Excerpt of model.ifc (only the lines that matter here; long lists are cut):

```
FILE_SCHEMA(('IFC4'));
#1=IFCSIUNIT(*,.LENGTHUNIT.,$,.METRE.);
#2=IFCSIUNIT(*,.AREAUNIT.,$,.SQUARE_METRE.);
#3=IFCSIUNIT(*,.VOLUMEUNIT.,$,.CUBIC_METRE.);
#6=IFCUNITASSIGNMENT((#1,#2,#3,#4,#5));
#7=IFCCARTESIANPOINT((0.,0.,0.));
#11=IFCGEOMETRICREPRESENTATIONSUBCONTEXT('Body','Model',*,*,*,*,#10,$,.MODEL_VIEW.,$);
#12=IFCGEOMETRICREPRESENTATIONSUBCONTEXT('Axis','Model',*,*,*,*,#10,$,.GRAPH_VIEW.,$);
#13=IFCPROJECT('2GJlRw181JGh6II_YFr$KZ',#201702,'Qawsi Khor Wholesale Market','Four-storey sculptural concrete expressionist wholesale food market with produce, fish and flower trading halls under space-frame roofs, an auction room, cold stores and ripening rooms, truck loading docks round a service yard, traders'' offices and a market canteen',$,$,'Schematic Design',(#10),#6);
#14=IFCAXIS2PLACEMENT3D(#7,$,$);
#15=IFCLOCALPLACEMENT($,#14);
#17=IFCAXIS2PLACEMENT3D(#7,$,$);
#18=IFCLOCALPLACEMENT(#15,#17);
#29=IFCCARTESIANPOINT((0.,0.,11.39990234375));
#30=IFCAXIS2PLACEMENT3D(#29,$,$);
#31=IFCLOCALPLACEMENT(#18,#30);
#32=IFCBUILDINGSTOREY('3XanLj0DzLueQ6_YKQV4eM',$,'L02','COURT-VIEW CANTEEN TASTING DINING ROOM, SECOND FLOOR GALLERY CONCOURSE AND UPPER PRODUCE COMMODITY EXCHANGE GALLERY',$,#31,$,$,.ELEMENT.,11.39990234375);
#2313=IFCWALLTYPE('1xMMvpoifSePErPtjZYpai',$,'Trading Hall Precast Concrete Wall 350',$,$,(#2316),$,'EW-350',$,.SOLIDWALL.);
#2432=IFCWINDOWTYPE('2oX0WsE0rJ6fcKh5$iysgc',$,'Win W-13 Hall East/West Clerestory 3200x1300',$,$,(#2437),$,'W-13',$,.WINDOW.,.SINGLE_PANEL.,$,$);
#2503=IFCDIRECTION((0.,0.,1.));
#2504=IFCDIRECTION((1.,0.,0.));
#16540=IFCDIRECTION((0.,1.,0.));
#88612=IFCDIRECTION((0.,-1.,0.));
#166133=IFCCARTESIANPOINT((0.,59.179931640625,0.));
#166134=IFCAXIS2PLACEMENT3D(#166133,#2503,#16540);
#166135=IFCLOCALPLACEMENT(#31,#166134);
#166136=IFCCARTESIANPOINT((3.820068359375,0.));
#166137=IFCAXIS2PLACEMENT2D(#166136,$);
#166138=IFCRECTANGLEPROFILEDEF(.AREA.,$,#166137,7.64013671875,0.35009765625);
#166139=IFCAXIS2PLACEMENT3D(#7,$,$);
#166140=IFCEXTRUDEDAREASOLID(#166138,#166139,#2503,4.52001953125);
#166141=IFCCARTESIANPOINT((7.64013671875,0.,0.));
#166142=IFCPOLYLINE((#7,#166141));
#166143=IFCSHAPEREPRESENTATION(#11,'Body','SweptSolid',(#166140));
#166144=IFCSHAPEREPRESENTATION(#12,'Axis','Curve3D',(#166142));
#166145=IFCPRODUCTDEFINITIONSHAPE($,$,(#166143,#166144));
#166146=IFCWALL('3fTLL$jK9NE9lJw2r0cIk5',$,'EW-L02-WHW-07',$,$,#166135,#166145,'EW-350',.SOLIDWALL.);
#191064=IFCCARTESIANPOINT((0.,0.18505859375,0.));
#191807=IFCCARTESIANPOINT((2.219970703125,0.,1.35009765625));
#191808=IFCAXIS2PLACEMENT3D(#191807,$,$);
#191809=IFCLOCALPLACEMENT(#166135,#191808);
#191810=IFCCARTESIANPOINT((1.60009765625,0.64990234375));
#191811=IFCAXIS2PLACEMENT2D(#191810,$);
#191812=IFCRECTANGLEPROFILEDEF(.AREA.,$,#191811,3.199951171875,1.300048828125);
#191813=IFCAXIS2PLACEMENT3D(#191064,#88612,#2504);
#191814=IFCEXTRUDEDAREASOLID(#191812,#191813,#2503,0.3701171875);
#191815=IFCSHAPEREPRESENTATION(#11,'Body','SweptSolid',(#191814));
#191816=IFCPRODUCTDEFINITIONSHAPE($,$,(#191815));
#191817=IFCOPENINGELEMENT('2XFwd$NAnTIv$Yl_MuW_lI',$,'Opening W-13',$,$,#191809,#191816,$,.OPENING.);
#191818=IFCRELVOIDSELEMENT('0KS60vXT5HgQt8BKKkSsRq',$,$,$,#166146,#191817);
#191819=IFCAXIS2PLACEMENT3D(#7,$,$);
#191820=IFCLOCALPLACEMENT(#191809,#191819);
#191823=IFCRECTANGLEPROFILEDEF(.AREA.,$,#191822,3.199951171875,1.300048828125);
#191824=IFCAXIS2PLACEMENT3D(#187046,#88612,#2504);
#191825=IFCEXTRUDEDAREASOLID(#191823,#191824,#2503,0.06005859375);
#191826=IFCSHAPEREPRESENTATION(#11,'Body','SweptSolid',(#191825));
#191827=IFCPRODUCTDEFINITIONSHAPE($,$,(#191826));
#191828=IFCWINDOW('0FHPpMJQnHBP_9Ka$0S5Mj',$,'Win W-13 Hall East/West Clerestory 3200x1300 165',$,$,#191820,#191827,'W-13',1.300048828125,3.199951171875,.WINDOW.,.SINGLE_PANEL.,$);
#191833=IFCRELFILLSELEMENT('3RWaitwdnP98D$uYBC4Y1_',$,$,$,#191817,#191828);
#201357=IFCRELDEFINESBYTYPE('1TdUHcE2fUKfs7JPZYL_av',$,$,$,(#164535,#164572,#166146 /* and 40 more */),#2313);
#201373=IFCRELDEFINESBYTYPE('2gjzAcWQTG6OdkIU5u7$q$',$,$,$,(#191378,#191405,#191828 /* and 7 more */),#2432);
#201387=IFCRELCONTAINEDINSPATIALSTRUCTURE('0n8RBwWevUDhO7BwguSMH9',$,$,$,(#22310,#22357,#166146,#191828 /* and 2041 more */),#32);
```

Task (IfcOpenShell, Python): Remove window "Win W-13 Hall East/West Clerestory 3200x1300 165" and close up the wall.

```python
import ifcopenshell
import ifcopenshell.api.feature
import ifcopenshell.api.root
import ifcopenshell.geom
import ifcopenshell.util.shape

model = ifcopenshell.open("model.ifc")
settings = ifcopenshell.geom.settings()


def volume(element):
    """Net volume in cubic metres, openings subtracted."""
    shape = ifcopenshell.geom.create_shape(settings, element)
    return ifcopenshell.util.shape.get_volume(shape.geometry)


window = model.by_guid("0FHPpMJQnHBP_9Ka$0S5Mj")
opening = window.FillsVoids[0].RelatingOpeningElement
wall = opening.VoidsElements[0].RelatingBuildingElement
before = volume(wall)

ifcopenshell.api.root.remove_product(model, product=window)
ifcopenshell.api.feature.remove_feature(model, feature=opening)

after = volume(wall)

print(f"wall volume {before:.3f} -> {after:.3f} m3")

model.write("model_edited.ifc")
```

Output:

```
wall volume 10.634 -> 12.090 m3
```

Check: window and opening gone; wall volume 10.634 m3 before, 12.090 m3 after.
